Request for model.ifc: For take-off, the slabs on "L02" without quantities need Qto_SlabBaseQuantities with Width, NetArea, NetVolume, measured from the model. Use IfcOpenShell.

First a look at what the model holds.

```python
import ifcopenshell
import ifcopenshell.util.element
import ifcopenshell.util.unit

model = ifcopenshell.open("model.ifc")
print(model.schema)
for unit_type in ("LENGTHUNIT", "AREAUNIT", "VOLUMEUNIT"):
    print(unit_type, ifcopenshell.util.unit.calculate_unit_scale(model, unit_type))
storey = next(s for s in model.by_type("IfcBuildingStorey") if s.Name == "L02")
slabs = [e for e in ifcopenshell.util.element.get_decomposition(storey) if e.is_a("IfcSlab")]
for e in sorted(slabs, key=lambda e: e.id()):
    print(e.id(), e.is_a(), e.Name, list(ifcopenshell.util.element.get_psets(e, qtos_only=True)), sep=" | ")
```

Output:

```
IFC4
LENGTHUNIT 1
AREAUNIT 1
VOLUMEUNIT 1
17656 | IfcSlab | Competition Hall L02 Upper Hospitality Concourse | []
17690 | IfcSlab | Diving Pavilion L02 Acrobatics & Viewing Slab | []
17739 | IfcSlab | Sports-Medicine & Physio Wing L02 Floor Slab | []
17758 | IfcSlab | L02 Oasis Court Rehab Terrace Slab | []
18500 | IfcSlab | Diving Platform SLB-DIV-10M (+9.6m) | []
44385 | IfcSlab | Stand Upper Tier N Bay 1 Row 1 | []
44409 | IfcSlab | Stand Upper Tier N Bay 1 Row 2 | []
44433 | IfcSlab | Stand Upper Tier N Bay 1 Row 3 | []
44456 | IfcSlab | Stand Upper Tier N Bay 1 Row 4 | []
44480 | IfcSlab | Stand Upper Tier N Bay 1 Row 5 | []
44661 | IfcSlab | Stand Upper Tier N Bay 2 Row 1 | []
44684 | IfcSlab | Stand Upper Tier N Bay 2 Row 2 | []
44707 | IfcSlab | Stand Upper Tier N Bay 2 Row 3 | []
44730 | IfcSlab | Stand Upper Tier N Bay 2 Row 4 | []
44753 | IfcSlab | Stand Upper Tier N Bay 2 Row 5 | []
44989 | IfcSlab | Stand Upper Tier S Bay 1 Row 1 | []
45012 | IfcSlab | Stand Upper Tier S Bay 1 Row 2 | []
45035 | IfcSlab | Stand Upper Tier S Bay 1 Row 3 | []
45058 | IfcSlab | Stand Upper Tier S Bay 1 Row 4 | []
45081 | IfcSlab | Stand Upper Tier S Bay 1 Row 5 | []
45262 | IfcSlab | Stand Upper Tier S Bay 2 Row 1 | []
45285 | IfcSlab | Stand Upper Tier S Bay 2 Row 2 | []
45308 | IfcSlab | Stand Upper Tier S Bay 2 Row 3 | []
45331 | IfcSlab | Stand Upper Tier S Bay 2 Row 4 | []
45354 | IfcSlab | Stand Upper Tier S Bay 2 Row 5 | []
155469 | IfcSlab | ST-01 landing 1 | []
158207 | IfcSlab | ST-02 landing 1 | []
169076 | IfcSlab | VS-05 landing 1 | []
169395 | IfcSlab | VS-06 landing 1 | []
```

```python
import ifcopenshell
import ifcopenshell.api.pset
import ifcopenshell.geom
import ifcopenshell.util.element
import ifcopenshell.util.shape
import ifcopenshell.util.unit

model = ifcopenshell.open("model.ifc")
unit_scale = ifcopenshell.util.unit.calculate_unit_scale(model)
area_scale = ifcopenshell.util.unit.calculate_unit_scale(model, "AREAUNIT")
volume_scale = ifcopenshell.util.unit.calculate_unit_scale(model, "VOLUMEUNIT")
settings = ifcopenshell.geom.settings()

storey = next(s for s in model.by_type("IfcBuildingStorey") if s.Name == "L02")
slabs = [e for e in ifcopenshell.util.element.get_decomposition(storey) if e.is_a("IfcSlab")]

for e in sorted(slabs, key=lambda e: e.id()):
    if ifcopenshell.util.element.get_psets(e, qtos_only=True, should_inherit=False):
        continue
    # Geometry comes back in metres, in the element's own axes.
    shape = ifcopenshell.geom.create_shape(settings, e)
    values = {
        "Width": ifcopenshell.util.shape.get_z(shape.geometry) / unit_scale,
        "NetArea": ifcopenshell.util.shape.get_footprint_area(shape.geometry) / area_scale,
        "NetVolume": ifcopenshell.util.shape.get_volume(shape.geometry) / volume_scale,
    }
    qto = ifcopenshell.api.pset.add_qto(model, product=e, name="Qto_SlabBaseQuantities")
    ifcopenshell.api.pset.edit_qto(model, qto=qto, properties=values)
    print(e.id(), {k: round(v, 3) for k, v in values.items()})

model.write("model_rev.ifc")
```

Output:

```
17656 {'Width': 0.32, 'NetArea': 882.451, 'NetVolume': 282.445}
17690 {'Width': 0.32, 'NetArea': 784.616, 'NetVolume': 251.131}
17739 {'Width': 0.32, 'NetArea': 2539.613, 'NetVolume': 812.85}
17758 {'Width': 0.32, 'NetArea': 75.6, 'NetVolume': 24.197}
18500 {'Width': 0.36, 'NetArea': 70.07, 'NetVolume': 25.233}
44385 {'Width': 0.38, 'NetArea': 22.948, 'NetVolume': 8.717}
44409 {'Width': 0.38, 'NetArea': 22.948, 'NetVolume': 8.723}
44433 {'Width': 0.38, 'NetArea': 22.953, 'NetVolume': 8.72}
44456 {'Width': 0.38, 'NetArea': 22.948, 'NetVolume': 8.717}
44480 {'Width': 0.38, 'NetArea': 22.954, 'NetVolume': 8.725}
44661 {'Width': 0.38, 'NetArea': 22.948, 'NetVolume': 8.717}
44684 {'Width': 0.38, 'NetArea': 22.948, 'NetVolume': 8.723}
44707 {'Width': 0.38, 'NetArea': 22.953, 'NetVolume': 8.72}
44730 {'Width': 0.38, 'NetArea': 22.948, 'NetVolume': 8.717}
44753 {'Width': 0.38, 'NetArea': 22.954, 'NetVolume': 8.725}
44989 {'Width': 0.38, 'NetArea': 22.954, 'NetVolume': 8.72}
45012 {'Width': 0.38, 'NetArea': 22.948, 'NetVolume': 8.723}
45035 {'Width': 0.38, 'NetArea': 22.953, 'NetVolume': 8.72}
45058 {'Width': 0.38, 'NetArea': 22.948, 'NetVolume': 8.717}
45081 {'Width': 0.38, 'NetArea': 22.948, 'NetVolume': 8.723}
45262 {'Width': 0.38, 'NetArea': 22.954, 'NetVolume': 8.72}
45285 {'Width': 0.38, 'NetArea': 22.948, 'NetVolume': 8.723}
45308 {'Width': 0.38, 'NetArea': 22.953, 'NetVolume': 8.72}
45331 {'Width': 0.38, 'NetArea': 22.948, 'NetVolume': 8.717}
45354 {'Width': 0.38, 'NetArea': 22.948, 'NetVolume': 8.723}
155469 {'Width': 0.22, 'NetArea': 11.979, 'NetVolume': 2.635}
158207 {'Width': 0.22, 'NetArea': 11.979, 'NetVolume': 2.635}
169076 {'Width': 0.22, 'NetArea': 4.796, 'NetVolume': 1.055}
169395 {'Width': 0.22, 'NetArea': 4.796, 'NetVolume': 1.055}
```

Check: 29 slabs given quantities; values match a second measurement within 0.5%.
